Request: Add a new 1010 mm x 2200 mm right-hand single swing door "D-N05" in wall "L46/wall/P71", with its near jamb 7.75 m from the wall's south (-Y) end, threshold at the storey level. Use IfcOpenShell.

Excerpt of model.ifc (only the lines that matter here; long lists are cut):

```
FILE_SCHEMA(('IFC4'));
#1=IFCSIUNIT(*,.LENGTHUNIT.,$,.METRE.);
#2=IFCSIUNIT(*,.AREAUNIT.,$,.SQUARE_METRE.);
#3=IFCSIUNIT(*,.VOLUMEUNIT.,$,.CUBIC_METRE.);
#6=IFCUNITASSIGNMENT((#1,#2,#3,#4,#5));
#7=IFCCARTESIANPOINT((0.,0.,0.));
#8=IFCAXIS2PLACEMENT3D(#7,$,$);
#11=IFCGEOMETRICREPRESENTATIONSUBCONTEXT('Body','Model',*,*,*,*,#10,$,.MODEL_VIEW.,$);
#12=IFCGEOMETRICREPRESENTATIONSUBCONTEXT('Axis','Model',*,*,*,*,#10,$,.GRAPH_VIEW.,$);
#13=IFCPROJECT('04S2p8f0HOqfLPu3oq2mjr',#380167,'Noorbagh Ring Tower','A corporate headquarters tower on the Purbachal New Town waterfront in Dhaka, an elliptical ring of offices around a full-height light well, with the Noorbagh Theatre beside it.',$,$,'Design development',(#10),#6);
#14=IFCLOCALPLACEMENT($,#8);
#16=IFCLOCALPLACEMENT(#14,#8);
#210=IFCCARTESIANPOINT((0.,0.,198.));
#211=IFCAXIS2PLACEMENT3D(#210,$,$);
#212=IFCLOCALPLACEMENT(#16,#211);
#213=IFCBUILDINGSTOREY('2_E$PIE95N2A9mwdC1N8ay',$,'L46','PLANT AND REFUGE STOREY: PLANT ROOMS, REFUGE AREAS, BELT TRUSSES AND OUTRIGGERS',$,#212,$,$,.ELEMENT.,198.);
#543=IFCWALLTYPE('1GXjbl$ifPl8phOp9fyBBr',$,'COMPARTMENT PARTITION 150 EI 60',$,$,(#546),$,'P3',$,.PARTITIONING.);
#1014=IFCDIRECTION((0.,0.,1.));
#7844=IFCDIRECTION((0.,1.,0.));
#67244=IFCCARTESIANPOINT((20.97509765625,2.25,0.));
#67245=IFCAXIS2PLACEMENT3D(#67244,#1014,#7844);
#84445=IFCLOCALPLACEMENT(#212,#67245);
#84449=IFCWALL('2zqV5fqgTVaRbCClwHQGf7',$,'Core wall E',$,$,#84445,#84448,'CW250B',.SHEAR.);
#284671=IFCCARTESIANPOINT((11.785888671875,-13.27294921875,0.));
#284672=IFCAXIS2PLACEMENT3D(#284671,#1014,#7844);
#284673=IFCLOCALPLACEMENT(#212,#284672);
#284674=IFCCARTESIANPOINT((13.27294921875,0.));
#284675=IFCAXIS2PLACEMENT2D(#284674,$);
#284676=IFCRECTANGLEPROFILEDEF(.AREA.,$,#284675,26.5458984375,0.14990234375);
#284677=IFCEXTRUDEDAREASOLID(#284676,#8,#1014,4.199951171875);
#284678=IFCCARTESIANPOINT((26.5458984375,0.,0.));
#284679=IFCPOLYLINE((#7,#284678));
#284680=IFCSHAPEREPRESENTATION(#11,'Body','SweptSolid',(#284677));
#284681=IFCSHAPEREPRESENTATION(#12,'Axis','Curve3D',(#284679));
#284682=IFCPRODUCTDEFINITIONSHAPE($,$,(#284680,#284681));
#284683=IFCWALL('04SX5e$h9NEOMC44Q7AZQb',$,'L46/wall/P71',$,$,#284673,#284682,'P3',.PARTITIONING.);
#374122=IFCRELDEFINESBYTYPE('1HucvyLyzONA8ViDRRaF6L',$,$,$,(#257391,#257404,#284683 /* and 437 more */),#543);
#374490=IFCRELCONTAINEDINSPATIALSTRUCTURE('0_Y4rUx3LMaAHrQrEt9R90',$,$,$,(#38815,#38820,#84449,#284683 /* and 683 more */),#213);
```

```python
import numpy as np
import ifcopenshell
import ifcopenshell.api.feature
import ifcopenshell.api.geometry
import ifcopenshell.api.root
import ifcopenshell.api.spatial
import ifcopenshell.geom
import ifcopenshell.util.element
import ifcopenshell.util.placement
import ifcopenshell.util.representation
import ifcopenshell.util.shape
import ifcopenshell.util.unit

model = ifcopenshell.open("model.ifc")
unit_scale = ifcopenshell.util.unit.calculate_unit_scale(model)
settings = ifcopenshell.geom.settings()


def volume(element):
    """Net volume in cubic metres, openings subtracted."""
    shape = ifcopenshell.geom.create_shape(settings, element)
    return ifcopenshell.util.shape.get_volume(shape.geometry)


wall = model.by_guid("04SX5e$h9NEOMC44Q7AZQb")
storey = ifcopenshell.util.element.get_container(wall, ifc_class="IfcBuildingStorey")
context = ifcopenshell.util.representation.get_context(model, "Model", "Body", "MODEL_VIEW")
before = volume(wall)

width, height, from_end, sill = 1.01, 2.2, 7.75, 0.0  # metres

# The wall runs along its own X axis, and the end named is its -X end.
wall_shape = ifcopenshell.geom.create_shape(settings, wall)
x, y, z = ifcopenshell.util.shape.get_vertices(wall_shape.geometry).T
start = x.min() + from_end
face, thickness = float(y.min()), float(y.max() - y.min())
wall_matrix = ifcopenshell.util.placement.get_local_placement(wall.ObjectPlacement)
level = ifcopenshell.util.placement.get_local_placement(storey.ObjectPlacement)[2, 3]


def in_wall(x, y):
    """Placement at x, y metres in the wall's axes, at sill height."""
    matrix = wall_matrix.copy()
    matrix[:, 3] = wall_matrix @ np.array([x / unit_scale, y / unit_scale, 0.0, 1.0])
    matrix[2, 3] = level + sill / unit_scale
    return matrix


# Opening: a box that overshoots both wall faces by 50 mm.
opening = ifcopenshell.api.root.create_entity(model, ifc_class="IfcOpeningElement", predefined_type="OPENING")
box = ifcopenshell.api.geometry.add_wall_representation(
    model, context=context, length=width, height=height, thickness=thickness + 0.1
)
ifcopenshell.api.geometry.assign_representation(model, product=opening, representation=box)
ifcopenshell.api.geometry.edit_object_placement(model, product=opening, matrix=in_wall(start, face - 0.05), is_si=False)
ifcopenshell.api.feature.add_feature(model, feature=opening, element=wall)

door = ifcopenshell.api.root.create_entity(model, ifc_class="IfcDoor", name="D-N05", predefined_type="DOOR")
door.OverallWidth, door.OverallHeight = width / unit_scale, height / unit_scale
door.OperationType = "SINGLE_SWING_RIGHT"
body = ifcopenshell.api.geometry.add_door_representation(
    model,
    context=context,
    overall_width=door.OverallWidth,
    overall_height=door.OverallHeight,
    operation_type="SINGLE_SWING_RIGHT",
    lining_properties={"LiningDepth": thickness / unit_scale, "ThresholdDepth": thickness / unit_scale},
)
ifcopenshell.api.geometry.assign_representation(model, product=door, representation=body)
ifcopenshell.api.spatial.assign_container(model, products=[door], relating_structure=storey)
ifcopenshell.api.feature.add_filling(model, opening=opening, element=door)

# The lining spans the wall, so the door starts at the wall face.
ifcopenshell.api.geometry.edit_object_placement(model, product=door, matrix=in_wall(start, face), is_si=False)

after = volume(wall)

print(f"wall volume {before:.3f} -> {after:.3f} m3")

model.write("model-out.ifc")
```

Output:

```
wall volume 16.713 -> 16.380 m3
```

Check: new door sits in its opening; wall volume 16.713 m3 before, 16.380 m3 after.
